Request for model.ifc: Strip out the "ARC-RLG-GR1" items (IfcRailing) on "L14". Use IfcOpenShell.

First a look at what the model holds.

```python
import ifcopenshell
import ifcopenshell.util.element

model = ifcopenshell.open("model.ifc")
print(model.schema)
storey = next(s for s in model.by_type("IfcBuildingStorey") if s.Name == "L14")
railings = [e for e in ifcopenshell.util.element.get_decomposition(storey) if e.is_a("IfcRailing")]
seen = {}
for e in railings:
    element_type = ifcopenshell.util.element.get_type(e)
    name = element_type.Name if element_type not in (None, e) else None
    seen[name] = seen.get(name, 0) + 1
for name, count in sorted(seen.items(), key=str):
    print(count, "x", name)
```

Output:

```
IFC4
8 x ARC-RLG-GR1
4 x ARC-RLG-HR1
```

```python
import ifcopenshell
import ifcopenshell.api.root
import ifcopenshell.util.element

model = ifcopenshell.open("model.ifc")

storey = next(s for s in model.by_type("IfcBuildingStorey") if s.Name == "L14")
railings = [e for e in ifcopenshell.util.element.get_decomposition(storey) if e.is_a("IfcRailing")]
targets = [e for e in railings if (t := ifcopenshell.util.element.get_type(e)) not in (None, e) and t.Name == "ARC-RLG-GR1"]

for e in targets:
    ifcopenshell.api.root.remove_product(model, product=e)
print(len(targets), "removed")

model.write("model-out.ifc")
```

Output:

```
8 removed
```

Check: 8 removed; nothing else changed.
